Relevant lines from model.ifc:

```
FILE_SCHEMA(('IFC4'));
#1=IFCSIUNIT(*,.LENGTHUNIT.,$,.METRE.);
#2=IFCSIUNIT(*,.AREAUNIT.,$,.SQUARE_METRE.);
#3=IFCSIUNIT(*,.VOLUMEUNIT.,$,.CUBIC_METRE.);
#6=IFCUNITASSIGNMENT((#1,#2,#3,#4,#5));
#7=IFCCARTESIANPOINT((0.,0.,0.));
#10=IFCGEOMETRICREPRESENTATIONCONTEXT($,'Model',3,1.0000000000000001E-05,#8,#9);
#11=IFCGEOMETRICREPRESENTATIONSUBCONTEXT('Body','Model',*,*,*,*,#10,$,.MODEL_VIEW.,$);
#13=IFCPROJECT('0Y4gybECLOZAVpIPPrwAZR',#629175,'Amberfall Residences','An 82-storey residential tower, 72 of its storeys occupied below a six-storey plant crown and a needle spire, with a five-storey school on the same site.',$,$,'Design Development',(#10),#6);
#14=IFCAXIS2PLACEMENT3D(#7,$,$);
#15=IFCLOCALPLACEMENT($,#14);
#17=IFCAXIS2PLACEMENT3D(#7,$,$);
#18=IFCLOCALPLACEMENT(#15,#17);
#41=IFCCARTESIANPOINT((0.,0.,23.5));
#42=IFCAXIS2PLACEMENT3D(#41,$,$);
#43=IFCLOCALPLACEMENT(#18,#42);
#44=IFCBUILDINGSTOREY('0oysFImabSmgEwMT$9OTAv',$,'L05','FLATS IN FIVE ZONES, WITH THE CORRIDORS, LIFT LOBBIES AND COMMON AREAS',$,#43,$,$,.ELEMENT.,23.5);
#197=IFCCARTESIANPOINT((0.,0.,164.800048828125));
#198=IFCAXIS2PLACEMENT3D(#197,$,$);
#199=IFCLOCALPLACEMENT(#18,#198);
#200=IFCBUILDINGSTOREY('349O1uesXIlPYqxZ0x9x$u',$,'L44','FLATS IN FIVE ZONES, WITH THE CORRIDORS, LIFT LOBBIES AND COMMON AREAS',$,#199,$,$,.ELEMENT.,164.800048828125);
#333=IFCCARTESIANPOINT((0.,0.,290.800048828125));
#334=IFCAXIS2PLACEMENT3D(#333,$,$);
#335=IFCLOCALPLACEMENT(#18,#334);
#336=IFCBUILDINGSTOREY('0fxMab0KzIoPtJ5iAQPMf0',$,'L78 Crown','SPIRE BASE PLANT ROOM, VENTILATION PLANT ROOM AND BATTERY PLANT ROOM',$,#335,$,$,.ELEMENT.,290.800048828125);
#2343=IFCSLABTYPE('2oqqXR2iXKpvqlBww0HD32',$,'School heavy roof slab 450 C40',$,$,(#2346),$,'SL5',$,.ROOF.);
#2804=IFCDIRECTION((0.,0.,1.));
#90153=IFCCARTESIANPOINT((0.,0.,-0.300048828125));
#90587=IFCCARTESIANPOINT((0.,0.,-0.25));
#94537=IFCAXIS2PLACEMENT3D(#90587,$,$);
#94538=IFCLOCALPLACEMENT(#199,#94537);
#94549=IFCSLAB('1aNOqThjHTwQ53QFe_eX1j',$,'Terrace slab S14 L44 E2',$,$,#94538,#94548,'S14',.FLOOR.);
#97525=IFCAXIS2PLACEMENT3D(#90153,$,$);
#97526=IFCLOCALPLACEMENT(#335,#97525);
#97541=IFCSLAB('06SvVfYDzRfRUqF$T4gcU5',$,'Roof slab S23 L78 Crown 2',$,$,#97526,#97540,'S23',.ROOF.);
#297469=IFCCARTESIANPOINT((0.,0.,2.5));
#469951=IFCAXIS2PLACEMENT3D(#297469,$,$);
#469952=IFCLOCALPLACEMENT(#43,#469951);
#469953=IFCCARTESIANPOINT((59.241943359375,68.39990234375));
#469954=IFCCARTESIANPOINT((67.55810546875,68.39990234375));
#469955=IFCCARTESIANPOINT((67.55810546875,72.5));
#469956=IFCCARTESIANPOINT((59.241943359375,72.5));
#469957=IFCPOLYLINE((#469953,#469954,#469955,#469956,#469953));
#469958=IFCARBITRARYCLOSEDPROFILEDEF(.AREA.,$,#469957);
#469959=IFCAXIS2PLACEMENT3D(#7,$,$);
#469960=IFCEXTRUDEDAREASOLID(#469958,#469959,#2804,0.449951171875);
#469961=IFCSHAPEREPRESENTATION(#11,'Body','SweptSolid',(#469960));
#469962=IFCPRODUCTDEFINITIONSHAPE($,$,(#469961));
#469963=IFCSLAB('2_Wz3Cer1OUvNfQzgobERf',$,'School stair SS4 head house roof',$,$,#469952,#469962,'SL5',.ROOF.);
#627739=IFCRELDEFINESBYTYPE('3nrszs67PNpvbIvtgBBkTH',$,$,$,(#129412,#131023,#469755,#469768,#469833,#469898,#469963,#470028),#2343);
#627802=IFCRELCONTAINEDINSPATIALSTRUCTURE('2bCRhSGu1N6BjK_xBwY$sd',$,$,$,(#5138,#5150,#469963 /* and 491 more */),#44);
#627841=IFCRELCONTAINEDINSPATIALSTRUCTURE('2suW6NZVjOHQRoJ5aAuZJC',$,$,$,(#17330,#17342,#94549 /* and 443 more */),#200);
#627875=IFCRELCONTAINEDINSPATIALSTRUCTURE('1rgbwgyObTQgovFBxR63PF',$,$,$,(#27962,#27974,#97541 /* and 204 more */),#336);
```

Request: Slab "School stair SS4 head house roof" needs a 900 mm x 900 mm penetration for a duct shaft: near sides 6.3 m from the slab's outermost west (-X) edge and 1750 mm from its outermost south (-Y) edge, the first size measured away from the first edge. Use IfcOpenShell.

```python
import numpy as np
import ifcopenshell
import ifcopenshell.api.feature
import ifcopenshell.api.geometry
import ifcopenshell.api.root
import ifcopenshell.geom
import ifcopenshell.util.placement
import ifcopenshell.util.representation
import ifcopenshell.util.shape
import ifcopenshell.util.unit

model = ifcopenshell.open("model.ifc")
unit_scale = ifcopenshell.util.unit.calculate_unit_scale(model)
settings = ifcopenshell.geom.settings()


def volume(element):
    """Net volume in cubic metres, openings subtracted."""
    shape = ifcopenshell.geom.create_shape(settings, element)
    return ifcopenshell.util.shape.get_volume(shape.geometry)


slab = model.by_guid("2_Wz3Cer1OUvNfQzgobERf")
before = volume(slab)

# Extent in the slab's own axes, in metres. The edges named are its -X and -Y sides.
slab_shape = ifcopenshell.geom.create_shape(settings, slab)
vertices = ifcopenshell.util.shape.get_vertices(slab_shape.geometry)
x_min, y_min, bottom = vertices.min(axis=0)
top = vertices[:, 2].max()

opening = ifcopenshell.api.root.create_entity(model, ifc_class="IfcOpeningElement", name="Duct shaft opening", predefined_type="OPENING")
context = ifcopenshell.util.representation.get_context(model, "Model", "Body", "MODEL_VIEW")
width, depth = 0.9, 0.9
outline = [(0.0, 0.0), (width, 0.0), (width, depth), (0.0, depth), (0.0, 0.0)]
# Overshoot both faces by 50 mm so the cut is clean.
shape = ifcopenshell.api.geometry.add_slab_representation(
    model, context=context, depth=top - bottom + 0.1, polyline=outline
)
ifcopenshell.api.geometry.assign_representation(model, product=opening, representation=shape)

matrix = ifcopenshell.util.placement.get_local_placement(slab.ObjectPlacement)
matrix[:, 3] = matrix @ np.append(np.array([x_min + 6.3, y_min + 1.75, bottom - 0.05]) / unit_scale, 1.0)
ifcopenshell.api.geometry.edit_object_placement(model, product=opening, matrix=matrix, is_si=False)
ifcopenshell.api.feature.add_feature(model, feature=opening, element=slab)

after = volume(slab)

print(f"slab volume {before:.3f} -> {after:.3f} m3")

model.write("model_v2.ifc")
```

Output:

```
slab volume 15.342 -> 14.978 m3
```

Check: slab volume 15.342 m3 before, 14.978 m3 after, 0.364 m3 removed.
